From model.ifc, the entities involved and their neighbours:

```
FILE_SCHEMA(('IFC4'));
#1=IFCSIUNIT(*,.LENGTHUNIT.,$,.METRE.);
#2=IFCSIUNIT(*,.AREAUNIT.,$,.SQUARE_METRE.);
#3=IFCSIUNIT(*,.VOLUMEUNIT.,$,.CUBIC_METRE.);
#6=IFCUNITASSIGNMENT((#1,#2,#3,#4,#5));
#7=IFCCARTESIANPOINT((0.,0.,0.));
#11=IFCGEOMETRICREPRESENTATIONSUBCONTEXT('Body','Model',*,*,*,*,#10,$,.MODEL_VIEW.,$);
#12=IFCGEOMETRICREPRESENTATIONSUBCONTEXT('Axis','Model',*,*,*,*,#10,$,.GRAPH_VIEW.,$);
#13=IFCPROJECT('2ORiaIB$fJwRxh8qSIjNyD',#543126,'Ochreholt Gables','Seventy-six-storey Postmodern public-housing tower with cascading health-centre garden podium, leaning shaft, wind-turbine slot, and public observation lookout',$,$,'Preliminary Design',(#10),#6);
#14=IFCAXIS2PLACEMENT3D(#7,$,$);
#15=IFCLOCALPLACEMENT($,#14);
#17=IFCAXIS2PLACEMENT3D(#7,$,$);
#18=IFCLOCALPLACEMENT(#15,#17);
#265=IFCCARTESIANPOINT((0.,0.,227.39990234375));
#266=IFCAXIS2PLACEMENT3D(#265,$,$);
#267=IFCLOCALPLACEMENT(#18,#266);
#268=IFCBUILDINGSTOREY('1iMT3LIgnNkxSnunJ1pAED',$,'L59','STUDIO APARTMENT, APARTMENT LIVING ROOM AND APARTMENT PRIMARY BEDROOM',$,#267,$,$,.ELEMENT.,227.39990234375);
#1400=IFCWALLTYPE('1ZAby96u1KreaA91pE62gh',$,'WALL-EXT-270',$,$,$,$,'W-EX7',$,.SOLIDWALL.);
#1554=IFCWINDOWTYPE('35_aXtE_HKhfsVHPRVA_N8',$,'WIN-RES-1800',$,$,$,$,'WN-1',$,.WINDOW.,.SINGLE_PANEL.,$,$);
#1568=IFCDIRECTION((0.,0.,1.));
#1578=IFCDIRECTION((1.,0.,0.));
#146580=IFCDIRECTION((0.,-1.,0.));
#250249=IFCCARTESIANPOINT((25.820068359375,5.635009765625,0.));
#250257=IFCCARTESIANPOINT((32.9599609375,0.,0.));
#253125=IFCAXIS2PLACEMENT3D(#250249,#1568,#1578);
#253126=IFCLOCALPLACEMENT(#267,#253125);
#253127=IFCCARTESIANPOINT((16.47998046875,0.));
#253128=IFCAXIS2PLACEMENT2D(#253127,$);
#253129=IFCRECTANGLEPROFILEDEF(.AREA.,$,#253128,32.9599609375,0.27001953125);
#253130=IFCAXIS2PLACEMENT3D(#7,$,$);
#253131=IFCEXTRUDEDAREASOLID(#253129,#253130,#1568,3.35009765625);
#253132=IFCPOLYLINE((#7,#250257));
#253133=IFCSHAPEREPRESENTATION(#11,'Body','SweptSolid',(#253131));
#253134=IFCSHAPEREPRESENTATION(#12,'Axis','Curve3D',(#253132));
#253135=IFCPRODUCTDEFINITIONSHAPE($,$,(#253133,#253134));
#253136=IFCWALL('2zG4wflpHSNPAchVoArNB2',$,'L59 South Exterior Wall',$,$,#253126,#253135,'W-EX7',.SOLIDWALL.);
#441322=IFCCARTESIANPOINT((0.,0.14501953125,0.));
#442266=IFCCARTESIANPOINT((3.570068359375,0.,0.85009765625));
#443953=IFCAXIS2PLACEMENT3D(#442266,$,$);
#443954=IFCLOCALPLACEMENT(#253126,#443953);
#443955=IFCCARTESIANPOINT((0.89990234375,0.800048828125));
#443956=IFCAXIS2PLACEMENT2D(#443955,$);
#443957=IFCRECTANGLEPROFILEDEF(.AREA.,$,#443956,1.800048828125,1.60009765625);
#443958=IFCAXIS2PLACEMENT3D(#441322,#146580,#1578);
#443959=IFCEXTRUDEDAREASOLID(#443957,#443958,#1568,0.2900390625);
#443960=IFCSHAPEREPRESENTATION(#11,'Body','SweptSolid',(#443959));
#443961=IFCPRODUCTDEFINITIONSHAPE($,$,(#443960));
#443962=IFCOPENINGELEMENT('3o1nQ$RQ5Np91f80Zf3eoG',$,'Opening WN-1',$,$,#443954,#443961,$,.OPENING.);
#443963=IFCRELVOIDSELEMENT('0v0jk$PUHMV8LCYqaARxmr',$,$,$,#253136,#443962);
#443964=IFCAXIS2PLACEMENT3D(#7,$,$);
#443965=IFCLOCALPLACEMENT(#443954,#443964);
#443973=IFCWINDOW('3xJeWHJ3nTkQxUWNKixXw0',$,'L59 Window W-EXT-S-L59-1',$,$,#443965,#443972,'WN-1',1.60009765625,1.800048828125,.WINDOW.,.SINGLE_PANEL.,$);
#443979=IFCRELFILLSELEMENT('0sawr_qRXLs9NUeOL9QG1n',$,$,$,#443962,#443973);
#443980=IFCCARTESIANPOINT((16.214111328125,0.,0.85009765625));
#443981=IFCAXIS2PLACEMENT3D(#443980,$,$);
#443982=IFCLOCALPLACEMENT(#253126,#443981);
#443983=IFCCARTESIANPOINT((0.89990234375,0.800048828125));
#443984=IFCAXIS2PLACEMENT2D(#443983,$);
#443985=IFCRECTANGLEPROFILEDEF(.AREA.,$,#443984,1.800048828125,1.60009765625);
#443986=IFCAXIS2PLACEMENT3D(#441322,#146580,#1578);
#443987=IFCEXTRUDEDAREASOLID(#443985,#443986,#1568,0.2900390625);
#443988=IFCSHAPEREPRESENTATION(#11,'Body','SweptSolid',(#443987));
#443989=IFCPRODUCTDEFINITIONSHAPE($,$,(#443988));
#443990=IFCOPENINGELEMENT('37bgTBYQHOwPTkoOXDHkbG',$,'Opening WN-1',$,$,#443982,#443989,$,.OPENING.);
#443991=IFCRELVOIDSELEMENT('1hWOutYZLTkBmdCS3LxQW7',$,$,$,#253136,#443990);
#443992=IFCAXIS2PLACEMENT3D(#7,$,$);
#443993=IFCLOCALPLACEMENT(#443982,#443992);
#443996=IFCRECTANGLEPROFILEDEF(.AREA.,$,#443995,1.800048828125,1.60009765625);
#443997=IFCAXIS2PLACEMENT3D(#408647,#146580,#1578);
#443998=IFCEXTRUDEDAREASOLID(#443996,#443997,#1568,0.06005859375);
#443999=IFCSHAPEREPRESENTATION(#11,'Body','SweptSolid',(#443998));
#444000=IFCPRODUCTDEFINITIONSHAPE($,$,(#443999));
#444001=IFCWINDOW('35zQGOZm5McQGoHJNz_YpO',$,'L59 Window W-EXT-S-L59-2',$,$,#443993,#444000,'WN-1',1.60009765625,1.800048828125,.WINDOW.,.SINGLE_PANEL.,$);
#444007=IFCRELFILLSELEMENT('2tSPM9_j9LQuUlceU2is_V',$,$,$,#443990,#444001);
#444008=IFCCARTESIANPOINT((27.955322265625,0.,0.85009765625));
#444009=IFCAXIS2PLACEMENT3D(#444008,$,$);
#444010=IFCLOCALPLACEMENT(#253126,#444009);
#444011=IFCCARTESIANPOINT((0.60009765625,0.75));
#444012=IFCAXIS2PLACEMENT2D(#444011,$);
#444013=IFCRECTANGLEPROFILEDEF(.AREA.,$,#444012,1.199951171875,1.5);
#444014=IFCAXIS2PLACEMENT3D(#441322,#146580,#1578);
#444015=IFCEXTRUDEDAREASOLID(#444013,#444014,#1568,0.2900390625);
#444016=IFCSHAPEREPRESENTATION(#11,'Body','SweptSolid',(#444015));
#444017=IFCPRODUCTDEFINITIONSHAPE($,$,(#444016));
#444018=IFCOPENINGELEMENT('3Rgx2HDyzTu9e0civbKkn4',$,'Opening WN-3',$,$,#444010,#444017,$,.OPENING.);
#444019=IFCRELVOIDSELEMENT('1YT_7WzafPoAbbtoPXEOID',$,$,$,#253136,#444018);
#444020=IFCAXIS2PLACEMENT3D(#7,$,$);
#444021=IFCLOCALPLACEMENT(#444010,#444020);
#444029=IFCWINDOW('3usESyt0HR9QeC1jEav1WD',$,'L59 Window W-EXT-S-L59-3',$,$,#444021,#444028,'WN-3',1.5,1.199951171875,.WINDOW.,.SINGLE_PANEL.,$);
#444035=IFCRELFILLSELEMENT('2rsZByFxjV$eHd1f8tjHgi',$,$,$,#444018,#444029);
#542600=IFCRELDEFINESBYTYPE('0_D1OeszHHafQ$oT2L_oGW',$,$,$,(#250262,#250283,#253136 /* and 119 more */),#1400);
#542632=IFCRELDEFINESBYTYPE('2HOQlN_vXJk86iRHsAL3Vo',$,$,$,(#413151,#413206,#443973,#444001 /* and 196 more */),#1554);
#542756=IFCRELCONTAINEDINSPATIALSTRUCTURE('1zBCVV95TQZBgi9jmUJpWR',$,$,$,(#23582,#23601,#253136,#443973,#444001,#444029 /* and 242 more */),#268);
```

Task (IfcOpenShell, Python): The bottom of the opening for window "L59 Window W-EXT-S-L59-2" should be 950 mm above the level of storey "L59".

```python
import numpy as np
import ifcopenshell
import ifcopenshell.api.geometry
import ifcopenshell.geom
import ifcopenshell.util.element
import ifcopenshell.util.placement
import ifcopenshell.util.shape
import ifcopenshell.util.unit

model = ifcopenshell.open("model.ifc")
unit_scale = ifcopenshell.util.unit.calculate_unit_scale(model)

window = model.by_id(444001)
opening = window.FillsVoids[0].RelatingOpeningElement
storey = ifcopenshell.util.element.get_container(window, ifc_class="IfcBuildingStorey")
level = ifcopenshell.util.placement.get_local_placement(storey.ObjectPlacement)[2, 3]

# The opening's origin need not be at the sill, so measure its lowest point.
shape = ifcopenshell.geom.create_shape(ifcopenshell.geom.settings(), opening)
bottom = ifcopenshell.util.shape.get_shape_bottom_elevation(shape, shape.geometry) / unit_scale
dz = level + 0.95 / unit_scale - bottom

shift = np.array([0.0, 0.0, dz])
# The window is placed relative to its opening, so it follows when the opening moves.
matrix = ifcopenshell.util.placement.get_local_placement(opening.ObjectPlacement)
matrix[:3, 3] += shift
ifcopenshell.api.geometry.edit_object_placement(
    model, product=opening, matrix=matrix, is_si=False, should_transform_children=True
)

print(f"moved by {dz * unit_scale:+.3f} m")

model.write("model-out.ifc")
```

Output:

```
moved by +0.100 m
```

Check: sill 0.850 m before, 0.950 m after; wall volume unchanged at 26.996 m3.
